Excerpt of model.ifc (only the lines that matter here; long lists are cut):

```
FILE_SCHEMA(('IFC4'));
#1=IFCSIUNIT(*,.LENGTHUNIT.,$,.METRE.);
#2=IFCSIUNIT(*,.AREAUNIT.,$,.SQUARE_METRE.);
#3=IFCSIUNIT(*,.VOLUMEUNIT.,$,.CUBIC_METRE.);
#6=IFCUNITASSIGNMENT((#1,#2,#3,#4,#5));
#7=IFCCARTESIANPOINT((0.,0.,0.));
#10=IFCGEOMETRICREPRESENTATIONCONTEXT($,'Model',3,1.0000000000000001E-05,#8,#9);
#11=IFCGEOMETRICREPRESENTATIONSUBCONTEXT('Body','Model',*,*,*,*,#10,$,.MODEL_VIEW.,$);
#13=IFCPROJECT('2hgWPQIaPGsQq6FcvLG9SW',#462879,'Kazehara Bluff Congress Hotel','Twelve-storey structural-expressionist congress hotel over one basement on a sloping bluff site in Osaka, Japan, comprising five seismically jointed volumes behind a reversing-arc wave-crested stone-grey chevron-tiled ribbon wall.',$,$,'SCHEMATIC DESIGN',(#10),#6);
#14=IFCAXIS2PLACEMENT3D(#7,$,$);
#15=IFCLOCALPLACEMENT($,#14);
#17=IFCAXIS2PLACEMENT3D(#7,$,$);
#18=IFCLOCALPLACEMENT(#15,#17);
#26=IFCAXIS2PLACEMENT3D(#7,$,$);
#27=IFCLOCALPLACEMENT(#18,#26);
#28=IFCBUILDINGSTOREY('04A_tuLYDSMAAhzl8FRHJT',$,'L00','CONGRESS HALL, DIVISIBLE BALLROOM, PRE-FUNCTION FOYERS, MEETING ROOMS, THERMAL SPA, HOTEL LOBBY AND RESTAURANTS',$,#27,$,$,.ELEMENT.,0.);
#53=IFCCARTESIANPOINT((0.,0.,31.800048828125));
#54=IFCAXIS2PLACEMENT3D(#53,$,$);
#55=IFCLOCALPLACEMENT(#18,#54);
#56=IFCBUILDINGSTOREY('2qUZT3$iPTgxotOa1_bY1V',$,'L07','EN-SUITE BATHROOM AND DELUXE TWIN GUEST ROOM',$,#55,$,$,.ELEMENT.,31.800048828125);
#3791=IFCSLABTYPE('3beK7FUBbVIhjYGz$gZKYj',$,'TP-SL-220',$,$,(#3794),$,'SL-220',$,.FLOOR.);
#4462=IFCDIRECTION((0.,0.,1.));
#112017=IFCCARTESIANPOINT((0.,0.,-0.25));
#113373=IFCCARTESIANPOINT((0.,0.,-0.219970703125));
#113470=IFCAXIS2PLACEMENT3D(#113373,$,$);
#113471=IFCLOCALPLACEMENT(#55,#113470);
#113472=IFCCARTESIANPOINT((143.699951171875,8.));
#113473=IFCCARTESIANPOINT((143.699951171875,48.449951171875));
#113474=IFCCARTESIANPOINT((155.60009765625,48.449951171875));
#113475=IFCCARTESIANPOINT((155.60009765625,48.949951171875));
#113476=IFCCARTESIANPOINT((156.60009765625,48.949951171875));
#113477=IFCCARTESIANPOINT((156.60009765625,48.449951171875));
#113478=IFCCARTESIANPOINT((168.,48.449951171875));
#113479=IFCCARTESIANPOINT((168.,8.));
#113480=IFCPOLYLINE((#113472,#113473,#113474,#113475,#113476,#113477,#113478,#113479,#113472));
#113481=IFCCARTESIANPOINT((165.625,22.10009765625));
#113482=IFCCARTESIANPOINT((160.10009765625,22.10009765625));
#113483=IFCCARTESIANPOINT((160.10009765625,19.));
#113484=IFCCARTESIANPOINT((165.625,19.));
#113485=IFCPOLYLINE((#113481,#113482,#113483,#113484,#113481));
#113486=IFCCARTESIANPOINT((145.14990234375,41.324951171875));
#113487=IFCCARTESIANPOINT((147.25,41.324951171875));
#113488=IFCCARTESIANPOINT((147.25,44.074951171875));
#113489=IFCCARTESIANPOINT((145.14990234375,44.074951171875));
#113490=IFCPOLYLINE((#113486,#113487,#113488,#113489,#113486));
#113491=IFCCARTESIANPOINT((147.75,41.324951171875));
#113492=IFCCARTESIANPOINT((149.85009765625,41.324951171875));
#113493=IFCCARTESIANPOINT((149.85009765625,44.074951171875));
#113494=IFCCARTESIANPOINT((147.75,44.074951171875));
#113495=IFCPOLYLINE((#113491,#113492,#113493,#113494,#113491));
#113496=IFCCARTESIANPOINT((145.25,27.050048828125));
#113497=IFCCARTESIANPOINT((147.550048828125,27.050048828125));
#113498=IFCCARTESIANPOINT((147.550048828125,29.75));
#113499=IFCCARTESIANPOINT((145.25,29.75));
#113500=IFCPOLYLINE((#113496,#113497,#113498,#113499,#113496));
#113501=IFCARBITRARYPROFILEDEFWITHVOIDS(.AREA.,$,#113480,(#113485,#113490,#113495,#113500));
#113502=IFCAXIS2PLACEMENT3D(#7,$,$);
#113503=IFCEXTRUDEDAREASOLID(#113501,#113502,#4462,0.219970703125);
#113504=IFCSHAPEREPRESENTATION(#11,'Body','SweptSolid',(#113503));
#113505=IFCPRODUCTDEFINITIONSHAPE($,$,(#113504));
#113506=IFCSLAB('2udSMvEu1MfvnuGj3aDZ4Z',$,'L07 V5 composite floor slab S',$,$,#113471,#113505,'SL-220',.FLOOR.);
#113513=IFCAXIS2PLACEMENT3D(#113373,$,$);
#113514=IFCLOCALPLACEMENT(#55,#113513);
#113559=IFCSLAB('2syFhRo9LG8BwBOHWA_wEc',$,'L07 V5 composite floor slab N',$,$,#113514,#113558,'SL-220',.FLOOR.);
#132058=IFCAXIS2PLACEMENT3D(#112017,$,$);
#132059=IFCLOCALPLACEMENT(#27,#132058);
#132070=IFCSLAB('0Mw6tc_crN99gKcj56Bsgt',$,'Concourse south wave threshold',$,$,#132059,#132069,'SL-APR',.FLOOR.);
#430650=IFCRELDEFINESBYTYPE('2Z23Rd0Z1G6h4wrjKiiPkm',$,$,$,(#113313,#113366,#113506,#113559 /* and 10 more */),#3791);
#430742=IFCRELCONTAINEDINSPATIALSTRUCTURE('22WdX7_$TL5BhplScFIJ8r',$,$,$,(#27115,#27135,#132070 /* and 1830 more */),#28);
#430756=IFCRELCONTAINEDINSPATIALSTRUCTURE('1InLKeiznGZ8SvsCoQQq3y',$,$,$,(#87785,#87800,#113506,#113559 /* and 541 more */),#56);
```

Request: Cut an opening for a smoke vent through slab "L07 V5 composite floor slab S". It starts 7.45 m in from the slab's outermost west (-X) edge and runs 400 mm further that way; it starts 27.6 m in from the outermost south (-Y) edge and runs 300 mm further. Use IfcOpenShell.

```python
import numpy as np
import ifcopenshell
import ifcopenshell.api.feature
import ifcopenshell.api.geometry
import ifcopenshell.api.root
import ifcopenshell.geom
import ifcopenshell.util.placement
import ifcopenshell.util.representation
import ifcopenshell.util.shape
import ifcopenshell.util.unit

model = ifcopenshell.open("model.ifc")
unit_scale = ifcopenshell.util.unit.calculate_unit_scale(model)
settings = ifcopenshell.geom.settings()


def volume(element):
    """Net volume in cubic metres, openings subtracted."""
    shape = ifcopenshell.geom.create_shape(settings, element)
    return ifcopenshell.util.shape.get_volume(shape.geometry)


slab = model.by_guid("2udSMvEu1MfvnuGj3aDZ4Z")
before = volume(slab)

# Extent in the slab's own axes, in metres. The edges named are its -X and -Y sides.
slab_shape = ifcopenshell.geom.create_shape(settings, slab)
vertices = ifcopenshell.util.shape.get_vertices(slab_shape.geometry)
x_min, y_min, bottom = vertices.min(axis=0)
top = vertices[:, 2].max()

opening = ifcopenshell.api.root.create_entity(model, ifc_class="IfcOpeningElement", name="Smoke vent opening", predefined_type="OPENING")
context = ifcopenshell.util.representation.get_context(model, "Model", "Body", "MODEL_VIEW")
width, depth = 0.4, 0.3
outline = [(0.0, 0.0), (width, 0.0), (width, depth), (0.0, depth), (0.0, 0.0)]
# Overshoot both faces by 50 mm so the cut is clean.
shape = ifcopenshell.api.geometry.add_slab_representation(
    model, context=context, depth=top - bottom + 0.1, polyline=outline
)
ifcopenshell.api.geometry.assign_representation(model, product=opening, representation=shape)

matrix = ifcopenshell.util.placement.get_local_placement(slab.ObjectPlacement)
matrix[:, 3] = matrix @ np.append(np.array([x_min + 7.45, y_min + 27.6, bottom - 0.05]) / unit_scale, 1.0)
ifcopenshell.api.geometry.edit_object_placement(model, product=opening, matrix=matrix, is_si=False)
ifcopenshell.api.feature.add_feature(model, feature=opening, element=slab)

after = volume(slab)

print(f"slab volume {before:.3f} -> {after:.3f} m3")

model.write("model-out.ifc")
```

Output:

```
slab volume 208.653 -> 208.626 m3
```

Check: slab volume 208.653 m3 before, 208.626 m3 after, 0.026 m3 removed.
